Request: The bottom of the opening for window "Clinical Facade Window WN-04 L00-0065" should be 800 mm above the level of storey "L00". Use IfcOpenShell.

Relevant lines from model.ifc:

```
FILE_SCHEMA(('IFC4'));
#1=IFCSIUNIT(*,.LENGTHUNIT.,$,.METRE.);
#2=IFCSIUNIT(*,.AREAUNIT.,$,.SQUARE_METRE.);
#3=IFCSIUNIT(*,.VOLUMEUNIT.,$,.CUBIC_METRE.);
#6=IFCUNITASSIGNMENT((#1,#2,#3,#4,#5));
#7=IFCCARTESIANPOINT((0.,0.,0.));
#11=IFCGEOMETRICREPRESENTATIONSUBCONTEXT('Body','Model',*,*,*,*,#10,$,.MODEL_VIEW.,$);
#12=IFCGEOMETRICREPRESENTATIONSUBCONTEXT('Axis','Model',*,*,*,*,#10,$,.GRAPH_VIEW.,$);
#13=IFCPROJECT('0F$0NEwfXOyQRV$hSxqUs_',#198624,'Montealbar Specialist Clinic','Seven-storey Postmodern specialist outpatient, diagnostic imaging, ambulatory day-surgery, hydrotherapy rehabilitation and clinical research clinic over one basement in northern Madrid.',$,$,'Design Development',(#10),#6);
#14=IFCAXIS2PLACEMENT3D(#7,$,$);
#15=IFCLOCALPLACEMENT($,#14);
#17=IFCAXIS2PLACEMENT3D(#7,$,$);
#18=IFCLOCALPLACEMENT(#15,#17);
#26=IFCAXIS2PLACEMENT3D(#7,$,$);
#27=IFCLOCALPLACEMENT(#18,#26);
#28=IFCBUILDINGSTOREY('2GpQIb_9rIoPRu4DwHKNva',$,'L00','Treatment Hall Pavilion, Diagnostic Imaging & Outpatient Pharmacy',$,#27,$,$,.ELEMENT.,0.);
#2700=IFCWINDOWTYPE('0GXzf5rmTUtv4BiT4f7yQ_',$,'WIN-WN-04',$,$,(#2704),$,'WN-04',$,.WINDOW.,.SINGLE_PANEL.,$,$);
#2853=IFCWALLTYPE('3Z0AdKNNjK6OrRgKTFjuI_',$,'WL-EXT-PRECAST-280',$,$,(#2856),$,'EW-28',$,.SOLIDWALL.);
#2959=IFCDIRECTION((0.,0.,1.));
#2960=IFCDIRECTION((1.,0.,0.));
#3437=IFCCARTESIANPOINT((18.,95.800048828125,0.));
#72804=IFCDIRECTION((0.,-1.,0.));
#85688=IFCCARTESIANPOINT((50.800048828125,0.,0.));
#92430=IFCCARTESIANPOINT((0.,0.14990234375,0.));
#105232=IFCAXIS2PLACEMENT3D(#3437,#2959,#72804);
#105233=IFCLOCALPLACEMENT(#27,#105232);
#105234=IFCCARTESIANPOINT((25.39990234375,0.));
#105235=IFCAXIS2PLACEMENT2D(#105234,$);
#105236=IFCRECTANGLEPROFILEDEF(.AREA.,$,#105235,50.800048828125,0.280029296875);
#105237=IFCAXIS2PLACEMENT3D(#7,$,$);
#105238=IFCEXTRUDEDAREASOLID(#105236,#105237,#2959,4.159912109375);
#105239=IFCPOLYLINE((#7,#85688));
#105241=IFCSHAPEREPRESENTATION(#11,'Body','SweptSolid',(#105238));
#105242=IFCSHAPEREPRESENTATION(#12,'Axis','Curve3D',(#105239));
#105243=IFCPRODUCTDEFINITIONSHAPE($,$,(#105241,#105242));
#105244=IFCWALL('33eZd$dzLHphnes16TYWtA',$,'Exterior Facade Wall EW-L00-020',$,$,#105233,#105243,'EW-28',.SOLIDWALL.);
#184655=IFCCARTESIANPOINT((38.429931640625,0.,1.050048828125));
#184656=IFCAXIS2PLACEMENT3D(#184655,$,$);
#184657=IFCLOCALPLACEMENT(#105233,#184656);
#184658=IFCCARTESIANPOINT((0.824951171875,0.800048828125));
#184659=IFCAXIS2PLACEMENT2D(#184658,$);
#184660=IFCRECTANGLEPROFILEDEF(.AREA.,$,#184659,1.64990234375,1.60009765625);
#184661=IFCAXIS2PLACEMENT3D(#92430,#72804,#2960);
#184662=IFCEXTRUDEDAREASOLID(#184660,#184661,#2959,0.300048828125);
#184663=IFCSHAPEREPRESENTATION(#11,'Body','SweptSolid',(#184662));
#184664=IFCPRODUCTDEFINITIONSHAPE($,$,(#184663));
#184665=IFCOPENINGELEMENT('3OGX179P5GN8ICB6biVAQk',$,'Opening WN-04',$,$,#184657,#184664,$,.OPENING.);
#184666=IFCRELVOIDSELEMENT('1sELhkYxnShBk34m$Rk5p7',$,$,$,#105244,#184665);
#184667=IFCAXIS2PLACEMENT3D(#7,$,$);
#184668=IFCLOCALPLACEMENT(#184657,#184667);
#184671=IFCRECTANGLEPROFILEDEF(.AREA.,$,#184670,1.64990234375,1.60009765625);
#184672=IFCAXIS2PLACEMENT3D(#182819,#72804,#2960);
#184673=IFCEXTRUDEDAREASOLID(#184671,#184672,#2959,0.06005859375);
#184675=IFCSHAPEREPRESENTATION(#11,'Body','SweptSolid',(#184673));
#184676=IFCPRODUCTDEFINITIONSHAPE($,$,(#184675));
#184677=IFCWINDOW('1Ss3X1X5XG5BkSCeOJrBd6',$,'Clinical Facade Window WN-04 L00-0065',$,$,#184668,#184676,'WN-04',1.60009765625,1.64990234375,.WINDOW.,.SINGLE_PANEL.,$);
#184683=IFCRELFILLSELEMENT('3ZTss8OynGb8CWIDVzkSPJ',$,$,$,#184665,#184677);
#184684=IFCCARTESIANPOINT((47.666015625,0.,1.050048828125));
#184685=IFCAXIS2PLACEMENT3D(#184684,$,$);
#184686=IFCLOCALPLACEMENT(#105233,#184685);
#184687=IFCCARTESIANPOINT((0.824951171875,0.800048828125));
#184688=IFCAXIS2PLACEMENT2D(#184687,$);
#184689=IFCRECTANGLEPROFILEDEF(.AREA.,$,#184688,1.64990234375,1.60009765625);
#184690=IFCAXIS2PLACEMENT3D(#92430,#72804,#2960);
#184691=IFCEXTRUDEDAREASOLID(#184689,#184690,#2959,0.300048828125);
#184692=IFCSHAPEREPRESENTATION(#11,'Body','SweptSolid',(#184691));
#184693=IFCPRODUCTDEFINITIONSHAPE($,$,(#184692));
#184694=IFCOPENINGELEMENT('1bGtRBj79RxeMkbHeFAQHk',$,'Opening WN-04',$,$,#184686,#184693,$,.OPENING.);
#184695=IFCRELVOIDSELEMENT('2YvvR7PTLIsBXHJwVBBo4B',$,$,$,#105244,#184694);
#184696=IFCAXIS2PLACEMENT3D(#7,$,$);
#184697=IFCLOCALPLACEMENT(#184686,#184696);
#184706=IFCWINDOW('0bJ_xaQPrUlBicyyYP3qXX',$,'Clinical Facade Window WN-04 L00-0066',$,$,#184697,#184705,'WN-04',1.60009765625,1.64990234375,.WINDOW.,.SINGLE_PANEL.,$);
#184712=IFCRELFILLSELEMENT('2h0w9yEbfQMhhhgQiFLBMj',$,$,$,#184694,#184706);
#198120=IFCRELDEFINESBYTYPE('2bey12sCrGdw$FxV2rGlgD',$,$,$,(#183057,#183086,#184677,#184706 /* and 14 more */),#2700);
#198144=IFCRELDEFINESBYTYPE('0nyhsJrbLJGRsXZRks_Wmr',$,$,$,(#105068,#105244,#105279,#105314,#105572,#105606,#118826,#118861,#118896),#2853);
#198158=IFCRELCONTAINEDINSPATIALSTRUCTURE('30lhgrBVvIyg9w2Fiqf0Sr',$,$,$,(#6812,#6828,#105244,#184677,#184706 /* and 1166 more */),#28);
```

```python
import numpy as np
import ifcopenshell
import ifcopenshell.api.geometry
import ifcopenshell.geom
import ifcopenshell.util.element
import ifcopenshell.util.placement
import ifcopenshell.util.shape
import ifcopenshell.util.unit

model = ifcopenshell.open("model.ifc")
unit_scale = ifcopenshell.util.unit.calculate_unit_scale(model)

window = model.by_guid("1Ss3X1X5XG5BkSCeOJrBd6")
opening = window.FillsVoids[0].RelatingOpeningElement
storey = ifcopenshell.util.element.get_container(window, ifc_class="IfcBuildingStorey")
level = ifcopenshell.util.placement.get_local_placement(storey.ObjectPlacement)[2, 3]

# The opening's origin need not be at the sill, so measure its lowest point.
shape = ifcopenshell.geom.create_shape(ifcopenshell.geom.settings(), opening)
bottom = ifcopenshell.util.shape.get_shape_bottom_elevation(shape, shape.geometry) / unit_scale
dz = level + 0.8 / unit_scale - bottom

shift = np.array([0.0, 0.0, dz])
# The window is placed relative to its opening, so it follows when the opening moves.
matrix = ifcopenshell.util.placement.get_local_placement(opening.ObjectPlacement)
matrix[:3, 3] += shift
ifcopenshell.api.geometry.edit_object_placement(
    model, product=opening, matrix=matrix, is_si=False, should_transform_children=True
)

print(f"moved by {dz * unit_scale:+.3f} m")

model.write("model_updated.ifc")
```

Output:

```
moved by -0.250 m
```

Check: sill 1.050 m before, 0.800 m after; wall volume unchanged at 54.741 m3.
